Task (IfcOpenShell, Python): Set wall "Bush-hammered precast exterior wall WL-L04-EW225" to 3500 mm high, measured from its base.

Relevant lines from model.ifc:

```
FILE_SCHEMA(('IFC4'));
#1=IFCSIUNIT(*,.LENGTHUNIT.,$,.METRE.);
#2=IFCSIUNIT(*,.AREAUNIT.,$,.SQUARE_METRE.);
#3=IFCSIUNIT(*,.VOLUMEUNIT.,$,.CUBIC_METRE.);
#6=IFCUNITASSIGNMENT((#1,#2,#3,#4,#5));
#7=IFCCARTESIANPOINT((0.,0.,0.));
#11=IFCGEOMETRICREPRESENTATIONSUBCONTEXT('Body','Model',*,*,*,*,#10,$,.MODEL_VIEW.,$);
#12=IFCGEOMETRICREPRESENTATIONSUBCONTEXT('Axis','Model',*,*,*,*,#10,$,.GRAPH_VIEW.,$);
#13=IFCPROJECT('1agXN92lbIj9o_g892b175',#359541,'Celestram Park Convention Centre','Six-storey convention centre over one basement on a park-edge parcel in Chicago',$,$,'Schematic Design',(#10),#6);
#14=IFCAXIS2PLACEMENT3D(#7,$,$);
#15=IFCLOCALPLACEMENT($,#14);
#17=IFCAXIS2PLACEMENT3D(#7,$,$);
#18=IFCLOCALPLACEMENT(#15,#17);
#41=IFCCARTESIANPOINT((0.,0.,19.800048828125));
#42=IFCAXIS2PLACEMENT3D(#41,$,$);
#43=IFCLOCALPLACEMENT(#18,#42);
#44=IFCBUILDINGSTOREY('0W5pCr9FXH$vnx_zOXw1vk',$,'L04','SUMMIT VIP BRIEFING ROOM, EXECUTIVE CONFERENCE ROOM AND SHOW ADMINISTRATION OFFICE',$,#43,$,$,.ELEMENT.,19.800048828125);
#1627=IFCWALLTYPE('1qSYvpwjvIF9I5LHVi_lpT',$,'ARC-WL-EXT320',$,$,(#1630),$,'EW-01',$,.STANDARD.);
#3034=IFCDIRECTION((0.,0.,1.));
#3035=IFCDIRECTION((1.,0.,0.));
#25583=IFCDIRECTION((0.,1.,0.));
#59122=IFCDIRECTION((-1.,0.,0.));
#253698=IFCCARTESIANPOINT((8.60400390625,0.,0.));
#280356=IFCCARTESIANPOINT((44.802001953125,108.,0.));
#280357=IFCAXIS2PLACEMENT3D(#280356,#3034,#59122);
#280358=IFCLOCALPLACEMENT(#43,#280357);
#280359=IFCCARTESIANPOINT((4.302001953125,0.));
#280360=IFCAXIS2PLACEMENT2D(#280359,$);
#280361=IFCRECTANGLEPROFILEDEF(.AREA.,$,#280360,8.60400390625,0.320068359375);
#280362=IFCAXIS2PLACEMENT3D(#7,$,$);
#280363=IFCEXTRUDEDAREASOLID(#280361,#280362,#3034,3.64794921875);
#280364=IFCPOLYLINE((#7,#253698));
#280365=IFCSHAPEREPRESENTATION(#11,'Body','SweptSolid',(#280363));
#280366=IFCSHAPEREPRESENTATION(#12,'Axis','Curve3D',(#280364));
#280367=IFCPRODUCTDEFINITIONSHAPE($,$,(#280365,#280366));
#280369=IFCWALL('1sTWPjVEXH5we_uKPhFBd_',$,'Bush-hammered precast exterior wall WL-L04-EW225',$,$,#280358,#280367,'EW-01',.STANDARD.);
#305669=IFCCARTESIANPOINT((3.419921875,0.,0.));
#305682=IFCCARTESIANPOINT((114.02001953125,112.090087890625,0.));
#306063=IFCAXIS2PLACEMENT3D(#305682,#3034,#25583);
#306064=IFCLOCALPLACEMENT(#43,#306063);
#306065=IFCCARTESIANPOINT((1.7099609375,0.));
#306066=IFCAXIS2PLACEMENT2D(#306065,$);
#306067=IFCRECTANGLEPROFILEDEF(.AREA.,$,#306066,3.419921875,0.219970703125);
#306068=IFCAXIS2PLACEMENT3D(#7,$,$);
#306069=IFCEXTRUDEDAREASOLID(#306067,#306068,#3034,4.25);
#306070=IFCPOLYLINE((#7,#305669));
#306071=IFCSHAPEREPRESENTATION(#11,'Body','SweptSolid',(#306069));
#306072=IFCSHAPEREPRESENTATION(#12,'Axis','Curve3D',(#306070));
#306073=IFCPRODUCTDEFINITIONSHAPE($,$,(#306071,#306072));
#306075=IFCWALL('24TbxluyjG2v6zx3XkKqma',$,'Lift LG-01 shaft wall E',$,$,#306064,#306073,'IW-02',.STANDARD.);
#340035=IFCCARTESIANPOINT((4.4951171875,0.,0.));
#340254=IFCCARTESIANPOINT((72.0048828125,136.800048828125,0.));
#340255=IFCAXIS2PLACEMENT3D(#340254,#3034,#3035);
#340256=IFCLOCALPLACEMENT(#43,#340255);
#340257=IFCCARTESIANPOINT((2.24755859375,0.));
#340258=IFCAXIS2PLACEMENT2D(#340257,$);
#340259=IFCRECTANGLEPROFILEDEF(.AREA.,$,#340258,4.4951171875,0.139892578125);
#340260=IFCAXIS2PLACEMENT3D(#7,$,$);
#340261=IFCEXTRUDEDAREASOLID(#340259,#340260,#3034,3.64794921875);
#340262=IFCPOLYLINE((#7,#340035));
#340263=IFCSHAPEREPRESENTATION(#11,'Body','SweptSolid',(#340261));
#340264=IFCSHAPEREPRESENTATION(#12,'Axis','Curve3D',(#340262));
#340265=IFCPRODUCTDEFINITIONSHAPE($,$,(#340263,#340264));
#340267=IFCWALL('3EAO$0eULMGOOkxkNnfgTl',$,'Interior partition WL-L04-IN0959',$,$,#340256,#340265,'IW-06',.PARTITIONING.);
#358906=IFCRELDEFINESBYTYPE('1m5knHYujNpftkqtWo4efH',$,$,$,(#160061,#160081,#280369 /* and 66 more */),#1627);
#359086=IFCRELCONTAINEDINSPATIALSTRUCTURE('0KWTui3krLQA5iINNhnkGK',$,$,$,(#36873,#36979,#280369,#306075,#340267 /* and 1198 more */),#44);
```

```python
import ifcopenshell
import ifcopenshell.geom
import ifcopenshell.util.representation
import ifcopenshell.util.shape
import ifcopenshell.util.unit

model = ifcopenshell.open("model.ifc")
unit_scale = ifcopenshell.util.unit.calculate_unit_scale(model)
settings = ifcopenshell.geom.settings()


def volume(element):
    """Net volume in cubic metres, openings subtracted."""
    shape = ifcopenshell.geom.create_shape(settings, element)
    return ifcopenshell.util.shape.get_volume(shape.geometry)


wall = model.by_guid("1sTWPjVEXH5we_uKPhFBd_")
before = volume(wall)

body = ifcopenshell.util.representation.get_representation(wall, "Model", "Body")
solid = body.Items[0]
old_height = solid.Depth
solid.Depth = 3.5 / unit_scale
after = volume(wall)

print(f"height {old_height:g} -> {solid.Depth:g}, volume {before:.3f} -> {after:.3f} m3")

model.write("model_edited.ifc")
```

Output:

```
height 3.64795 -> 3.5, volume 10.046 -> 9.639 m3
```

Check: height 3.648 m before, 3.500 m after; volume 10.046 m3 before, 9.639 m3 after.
